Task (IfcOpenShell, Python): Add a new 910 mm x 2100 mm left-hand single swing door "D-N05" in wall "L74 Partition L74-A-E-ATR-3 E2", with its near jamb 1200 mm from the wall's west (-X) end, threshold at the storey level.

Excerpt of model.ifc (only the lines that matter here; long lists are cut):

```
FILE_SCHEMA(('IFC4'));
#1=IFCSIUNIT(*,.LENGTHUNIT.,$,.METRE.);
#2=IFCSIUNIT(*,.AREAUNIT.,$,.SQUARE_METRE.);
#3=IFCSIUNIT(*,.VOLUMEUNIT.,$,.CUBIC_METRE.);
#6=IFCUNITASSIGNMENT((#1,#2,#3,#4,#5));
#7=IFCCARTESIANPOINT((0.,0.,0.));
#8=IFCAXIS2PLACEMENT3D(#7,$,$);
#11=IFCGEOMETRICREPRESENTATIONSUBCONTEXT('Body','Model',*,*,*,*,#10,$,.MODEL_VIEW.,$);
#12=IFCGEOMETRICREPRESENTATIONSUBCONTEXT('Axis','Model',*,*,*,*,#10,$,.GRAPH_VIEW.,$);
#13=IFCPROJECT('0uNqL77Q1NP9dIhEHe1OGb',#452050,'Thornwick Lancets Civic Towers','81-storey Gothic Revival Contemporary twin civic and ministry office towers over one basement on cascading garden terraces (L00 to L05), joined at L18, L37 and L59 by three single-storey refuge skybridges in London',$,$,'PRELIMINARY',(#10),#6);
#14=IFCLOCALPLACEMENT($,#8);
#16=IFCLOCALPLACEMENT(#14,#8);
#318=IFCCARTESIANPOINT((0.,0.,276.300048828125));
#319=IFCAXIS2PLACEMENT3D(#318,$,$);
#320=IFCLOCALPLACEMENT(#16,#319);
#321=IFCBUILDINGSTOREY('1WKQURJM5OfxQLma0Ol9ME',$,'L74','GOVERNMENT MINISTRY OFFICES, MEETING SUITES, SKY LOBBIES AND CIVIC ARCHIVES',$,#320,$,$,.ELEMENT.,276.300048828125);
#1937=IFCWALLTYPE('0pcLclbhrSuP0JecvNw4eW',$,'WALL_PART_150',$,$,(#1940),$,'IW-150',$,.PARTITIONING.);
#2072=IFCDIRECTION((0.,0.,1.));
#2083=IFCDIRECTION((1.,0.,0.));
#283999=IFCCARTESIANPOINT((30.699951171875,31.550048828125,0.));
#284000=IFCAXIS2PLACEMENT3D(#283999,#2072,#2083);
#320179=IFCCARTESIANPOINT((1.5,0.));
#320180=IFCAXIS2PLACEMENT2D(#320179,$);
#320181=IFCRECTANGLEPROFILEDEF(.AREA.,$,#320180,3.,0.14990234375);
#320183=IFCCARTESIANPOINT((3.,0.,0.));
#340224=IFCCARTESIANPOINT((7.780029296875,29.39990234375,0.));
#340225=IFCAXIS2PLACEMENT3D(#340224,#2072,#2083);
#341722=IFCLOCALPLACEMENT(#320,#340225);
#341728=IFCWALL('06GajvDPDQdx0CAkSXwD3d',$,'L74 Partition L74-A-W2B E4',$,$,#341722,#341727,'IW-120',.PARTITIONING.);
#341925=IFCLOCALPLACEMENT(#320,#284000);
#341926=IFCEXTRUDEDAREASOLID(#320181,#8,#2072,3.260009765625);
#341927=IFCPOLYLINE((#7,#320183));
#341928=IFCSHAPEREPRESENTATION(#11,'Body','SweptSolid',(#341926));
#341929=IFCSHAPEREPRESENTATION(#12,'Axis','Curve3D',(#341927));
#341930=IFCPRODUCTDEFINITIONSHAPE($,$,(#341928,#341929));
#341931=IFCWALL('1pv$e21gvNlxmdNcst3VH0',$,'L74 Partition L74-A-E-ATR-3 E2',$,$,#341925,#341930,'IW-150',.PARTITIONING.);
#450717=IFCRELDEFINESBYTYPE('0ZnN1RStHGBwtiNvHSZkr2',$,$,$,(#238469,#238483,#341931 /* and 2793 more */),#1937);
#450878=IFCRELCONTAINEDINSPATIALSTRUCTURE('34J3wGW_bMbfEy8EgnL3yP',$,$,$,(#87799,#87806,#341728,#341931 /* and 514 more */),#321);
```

```python
import numpy as np
import ifcopenshell
import ifcopenshell.api.feature
import ifcopenshell.api.geometry
import ifcopenshell.api.root
import ifcopenshell.api.spatial
import ifcopenshell.geom
import ifcopenshell.util.element
import ifcopenshell.util.placement
import ifcopenshell.util.representation
import ifcopenshell.util.shape
import ifcopenshell.util.unit

model = ifcopenshell.open("model.ifc")
unit_scale = ifcopenshell.util.unit.calculate_unit_scale(model)
settings = ifcopenshell.geom.settings()


def volume(element):
    """Net volume in cubic metres, openings subtracted."""
    shape = ifcopenshell.geom.create_shape(settings, element)
    return ifcopenshell.util.shape.get_volume(shape.geometry)


wall = model.by_guid("1pv$e21gvNlxmdNcst3VH0")
storey = ifcopenshell.util.element.get_container(wall, ifc_class="IfcBuildingStorey")
context = ifcopenshell.util.representation.get_context(model, "Model", "Body", "MODEL_VIEW")
before = volume(wall)

width, height, from_end, sill = 0.91, 2.1, 1.2, 0.0  # metres

# The wall runs along its own X axis, and the end named is its -X end.
wall_shape = ifcopenshell.geom.create_shape(settings, wall)
x, y, z = ifcopenshell.util.shape.get_vertices(wall_shape.geometry).T
start = x.min() + from_end
face, thickness = float(y.min()), float(y.max() - y.min())
wall_matrix = ifcopenshell.util.placement.get_local_placement(wall.ObjectPlacement)
level = ifcopenshell.util.placement.get_local_placement(storey.ObjectPlacement)[2, 3]


def in_wall(x, y):
    """Placement at x, y metres in the wall's axes, at sill height."""
    matrix = wall_matrix.copy()
    matrix[:, 3] = wall_matrix @ np.array([x / unit_scale, y / unit_scale, 0.0, 1.0])
    matrix[2, 3] = level + sill / unit_scale
    return matrix


# Opening: a box that overshoots both wall faces by 50 mm.
opening = ifcopenshell.api.root.create_entity(model, ifc_class="IfcOpeningElement", predefined_type="OPENING")
box = ifcopenshell.api.geometry.add_wall_representation(
    model, context=context, length=width, height=height, thickness=thickness + 0.1
)
ifcopenshell.api.geometry.assign_representation(model, product=opening, representation=box)
ifcopenshell.api.geometry.edit_object_placement(model, product=opening, matrix=in_wall(start, face - 0.05), is_si=False)
ifcopenshell.api.feature.add_feature(model, feature=opening, element=wall)

door = ifcopenshell.api.root.create_entity(model, ifc_class="IfcDoor", name="D-N05", predefined_type="DOOR")
door.OverallWidth, door.OverallHeight = width / unit_scale, height / unit_scale
door.OperationType = "SINGLE_SWING_LEFT"
body = ifcopenshell.api.geometry.add_door_representation(
    model,
    context=context,
    overall_width=door.OverallWidth,
    overall_height=door.OverallHeight,
    operation_type="SINGLE_SWING_LEFT",
    lining_properties={"LiningDepth": thickness / unit_scale, "ThresholdDepth": thickness / unit_scale},
)
ifcopenshell.api.geometry.assign_representation(model, product=door, representation=body)
ifcopenshell.api.spatial.assign_container(model, products=[door], relating_structure=storey)
ifcopenshell.api.feature.add_filling(model, opening=opening, element=door)

# The lining spans the wall, so the door starts at the wall face.
ifcopenshell.api.geometry.edit_object_placement(model, product=door, matrix=in_wall(start, face), is_si=False)

after = volume(wall)

print(f"wall volume {before:.3f} -> {after:.3f} m3")

model.write("model_v2.ifc")
```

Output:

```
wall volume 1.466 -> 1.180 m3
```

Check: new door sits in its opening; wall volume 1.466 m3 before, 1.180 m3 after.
